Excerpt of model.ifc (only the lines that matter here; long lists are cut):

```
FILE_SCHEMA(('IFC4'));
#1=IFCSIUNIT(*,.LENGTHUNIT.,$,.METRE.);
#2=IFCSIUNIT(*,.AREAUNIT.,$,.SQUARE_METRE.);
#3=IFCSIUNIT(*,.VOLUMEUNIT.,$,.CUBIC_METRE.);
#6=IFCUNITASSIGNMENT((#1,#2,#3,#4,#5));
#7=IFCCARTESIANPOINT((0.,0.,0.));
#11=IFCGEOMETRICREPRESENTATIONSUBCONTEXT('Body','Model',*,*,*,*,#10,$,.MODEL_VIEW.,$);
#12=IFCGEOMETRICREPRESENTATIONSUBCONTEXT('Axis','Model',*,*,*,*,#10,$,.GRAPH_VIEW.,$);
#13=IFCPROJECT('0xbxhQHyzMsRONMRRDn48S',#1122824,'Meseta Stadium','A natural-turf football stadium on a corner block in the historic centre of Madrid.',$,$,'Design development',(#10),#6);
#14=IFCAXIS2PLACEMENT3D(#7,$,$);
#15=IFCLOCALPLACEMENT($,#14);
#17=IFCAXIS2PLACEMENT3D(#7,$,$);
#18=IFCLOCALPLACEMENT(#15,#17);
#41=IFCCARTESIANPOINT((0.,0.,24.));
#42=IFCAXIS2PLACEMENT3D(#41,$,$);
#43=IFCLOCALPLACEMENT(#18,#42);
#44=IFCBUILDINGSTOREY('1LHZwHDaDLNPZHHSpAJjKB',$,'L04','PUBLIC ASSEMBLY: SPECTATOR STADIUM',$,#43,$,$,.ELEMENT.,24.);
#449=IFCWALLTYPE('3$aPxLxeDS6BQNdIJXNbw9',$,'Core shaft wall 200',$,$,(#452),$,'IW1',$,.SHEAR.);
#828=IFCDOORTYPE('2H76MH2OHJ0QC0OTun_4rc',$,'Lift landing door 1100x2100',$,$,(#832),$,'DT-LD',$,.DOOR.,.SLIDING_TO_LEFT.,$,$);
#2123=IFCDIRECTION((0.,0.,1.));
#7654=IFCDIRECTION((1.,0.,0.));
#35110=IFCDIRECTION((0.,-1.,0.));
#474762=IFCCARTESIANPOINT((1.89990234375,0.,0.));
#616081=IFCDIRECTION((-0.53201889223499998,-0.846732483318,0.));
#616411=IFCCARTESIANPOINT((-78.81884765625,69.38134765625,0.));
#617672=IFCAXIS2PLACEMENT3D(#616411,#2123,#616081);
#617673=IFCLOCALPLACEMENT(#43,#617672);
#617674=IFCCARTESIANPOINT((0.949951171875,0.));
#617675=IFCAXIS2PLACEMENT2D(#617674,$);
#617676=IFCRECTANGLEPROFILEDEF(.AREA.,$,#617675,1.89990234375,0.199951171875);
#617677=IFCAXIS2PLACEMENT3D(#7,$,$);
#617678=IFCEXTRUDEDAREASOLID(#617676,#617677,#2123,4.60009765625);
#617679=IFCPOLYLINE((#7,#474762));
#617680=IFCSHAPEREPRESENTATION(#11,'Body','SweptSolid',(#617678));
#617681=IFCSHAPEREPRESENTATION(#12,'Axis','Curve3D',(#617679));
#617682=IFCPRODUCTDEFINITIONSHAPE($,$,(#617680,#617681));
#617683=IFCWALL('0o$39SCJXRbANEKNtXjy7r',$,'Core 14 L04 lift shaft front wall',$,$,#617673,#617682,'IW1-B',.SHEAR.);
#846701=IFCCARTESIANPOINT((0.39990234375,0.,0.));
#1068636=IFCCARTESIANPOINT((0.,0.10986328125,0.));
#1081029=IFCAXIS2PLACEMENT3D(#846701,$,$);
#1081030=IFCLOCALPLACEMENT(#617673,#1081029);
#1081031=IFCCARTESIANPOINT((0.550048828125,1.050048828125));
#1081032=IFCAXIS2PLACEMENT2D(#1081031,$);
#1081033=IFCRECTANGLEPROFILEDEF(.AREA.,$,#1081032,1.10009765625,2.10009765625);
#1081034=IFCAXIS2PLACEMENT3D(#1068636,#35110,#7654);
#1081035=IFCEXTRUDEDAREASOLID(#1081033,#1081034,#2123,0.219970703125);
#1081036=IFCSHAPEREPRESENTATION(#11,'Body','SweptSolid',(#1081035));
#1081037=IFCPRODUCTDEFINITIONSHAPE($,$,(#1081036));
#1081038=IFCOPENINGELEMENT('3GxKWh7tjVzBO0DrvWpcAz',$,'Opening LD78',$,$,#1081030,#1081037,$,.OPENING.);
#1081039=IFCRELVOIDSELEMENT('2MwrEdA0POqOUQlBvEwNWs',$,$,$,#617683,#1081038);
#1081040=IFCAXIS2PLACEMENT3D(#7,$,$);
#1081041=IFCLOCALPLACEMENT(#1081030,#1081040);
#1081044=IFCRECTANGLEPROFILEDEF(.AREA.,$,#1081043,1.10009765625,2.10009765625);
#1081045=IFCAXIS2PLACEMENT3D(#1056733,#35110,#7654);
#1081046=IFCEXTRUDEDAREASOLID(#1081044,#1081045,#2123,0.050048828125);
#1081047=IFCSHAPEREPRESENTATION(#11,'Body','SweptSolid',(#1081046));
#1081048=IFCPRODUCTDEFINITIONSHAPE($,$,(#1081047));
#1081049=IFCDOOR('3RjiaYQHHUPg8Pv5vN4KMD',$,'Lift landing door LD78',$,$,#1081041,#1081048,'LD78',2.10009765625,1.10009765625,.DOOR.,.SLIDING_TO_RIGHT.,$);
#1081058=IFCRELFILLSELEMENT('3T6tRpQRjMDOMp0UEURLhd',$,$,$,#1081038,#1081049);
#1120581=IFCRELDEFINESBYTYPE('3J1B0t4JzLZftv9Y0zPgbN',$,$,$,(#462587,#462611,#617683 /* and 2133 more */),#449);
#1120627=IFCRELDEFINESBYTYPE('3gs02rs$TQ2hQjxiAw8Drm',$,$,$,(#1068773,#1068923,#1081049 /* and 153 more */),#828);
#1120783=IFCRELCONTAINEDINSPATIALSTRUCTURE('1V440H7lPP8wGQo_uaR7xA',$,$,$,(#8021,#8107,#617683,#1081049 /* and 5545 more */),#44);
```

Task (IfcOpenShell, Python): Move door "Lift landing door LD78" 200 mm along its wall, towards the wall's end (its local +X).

```python
import ifcopenshell
import ifcopenshell.api.geometry
import ifcopenshell.util.placement

model = ifcopenshell.open("model.ifc")

door = model.by_guid("3RjiaYQHHUPg8Pv5vN4KMD")
opening = door.FillsVoids[0].RelatingOpeningElement
wall = opening.VoidsElements[0].RelatingBuildingElement

wall_matrix = ifcopenshell.util.placement.get_local_placement(wall.ObjectPlacement)
shift = wall_matrix[:3, 0] * 0.2
before = ifcopenshell.util.placement.get_local_placement(door.ObjectPlacement)[:3, 3].copy()

# The door is placed relative to its opening, so it follows when the opening moves.
matrix = ifcopenshell.util.placement.get_local_placement(opening.ObjectPlacement)
matrix[:3, 3] += shift
ifcopenshell.api.geometry.edit_object_placement(
    model, product=opening, matrix=matrix, is_si=False, should_transform_children=True
)

after = ifcopenshell.util.placement.get_local_placement(door.ObjectPlacement)[:3, 3]
print("door moved by", (after - before).round(3) + 0.0)

model.write("model-out.ifc")
```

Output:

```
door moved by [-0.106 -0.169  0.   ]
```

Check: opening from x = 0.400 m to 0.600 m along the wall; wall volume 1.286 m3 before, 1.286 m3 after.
